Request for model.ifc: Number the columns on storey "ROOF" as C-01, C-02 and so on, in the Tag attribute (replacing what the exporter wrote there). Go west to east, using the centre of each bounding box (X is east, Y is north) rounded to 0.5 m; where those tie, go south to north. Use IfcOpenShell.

First a look at what the model holds.

```python
import ifcopenshell
import ifcopenshell.util.element
import ifcopenshell.util.placement

model = ifcopenshell.open("model.ifc")
print(model.schema)
storey = next(s for s in model.by_type("IfcBuildingStorey") if s.Name == "ROOF")
columns = [e for e in ifcopenshell.util.element.get_decomposition(storey) if e.is_a("IfcColumn")]
for e in sorted(columns, key=lambda e: e.id()):
    origin = ifcopenshell.util.placement.get_local_placement(e.ObjectPlacement)[:3, 3]
    print(e.id(), e.Tag, e.Name, origin.round(2) + 0.0, sep=" | ")
```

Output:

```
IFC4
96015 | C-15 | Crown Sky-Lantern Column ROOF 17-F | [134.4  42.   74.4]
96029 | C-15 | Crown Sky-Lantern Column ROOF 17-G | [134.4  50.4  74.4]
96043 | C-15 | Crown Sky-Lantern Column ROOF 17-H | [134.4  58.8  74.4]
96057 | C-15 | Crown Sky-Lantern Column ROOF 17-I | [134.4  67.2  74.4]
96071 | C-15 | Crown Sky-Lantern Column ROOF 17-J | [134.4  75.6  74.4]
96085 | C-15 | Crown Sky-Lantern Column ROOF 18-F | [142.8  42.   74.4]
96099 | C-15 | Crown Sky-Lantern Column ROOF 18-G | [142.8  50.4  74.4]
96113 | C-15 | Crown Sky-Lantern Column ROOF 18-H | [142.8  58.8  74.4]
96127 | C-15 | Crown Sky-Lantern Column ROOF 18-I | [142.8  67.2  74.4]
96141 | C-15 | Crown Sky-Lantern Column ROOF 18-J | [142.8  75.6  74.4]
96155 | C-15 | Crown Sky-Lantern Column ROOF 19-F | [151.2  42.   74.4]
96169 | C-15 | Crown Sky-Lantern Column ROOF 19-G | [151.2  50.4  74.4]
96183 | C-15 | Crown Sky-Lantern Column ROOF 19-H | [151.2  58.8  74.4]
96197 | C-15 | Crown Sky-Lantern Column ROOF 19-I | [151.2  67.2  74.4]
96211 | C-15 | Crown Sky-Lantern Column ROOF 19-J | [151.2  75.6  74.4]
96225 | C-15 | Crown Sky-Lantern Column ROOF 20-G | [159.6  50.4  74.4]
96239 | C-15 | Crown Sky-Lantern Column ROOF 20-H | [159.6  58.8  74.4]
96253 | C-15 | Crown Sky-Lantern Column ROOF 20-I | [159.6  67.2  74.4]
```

```python
import ifcopenshell
import ifcopenshell.geom
import ifcopenshell.util.element
import ifcopenshell.util.shape

model = ifcopenshell.open("model.ifc")
settings = ifcopenshell.geom.settings()
settings.set("use-world-coords", True)


def centre(element):
    shape = ifcopenshell.geom.create_shape(settings, element)
    return ifcopenshell.util.shape.get_bbox_centroid(shape.geometry)


storey = next(s for s in model.by_type("IfcBuildingStorey") if s.Name == "ROOF")
columns = [e for e in ifcopenshell.util.element.get_decomposition(storey) if e.is_a("IfcColumn")]

# Insertion points can sit at a corner or the storey origin, so sort by the geometry (in metres).
centres = {e: centre(e) for e in columns}
columns.sort(key=lambda e: (round(centres[e][0] / 0.5), centres[e][1]))

for i, e in enumerate(columns, start=1):
    number = f"C-{i:02d}"
    e.Tag = number
    print(e.id(), number)

model.write("model_edited.ifc")
```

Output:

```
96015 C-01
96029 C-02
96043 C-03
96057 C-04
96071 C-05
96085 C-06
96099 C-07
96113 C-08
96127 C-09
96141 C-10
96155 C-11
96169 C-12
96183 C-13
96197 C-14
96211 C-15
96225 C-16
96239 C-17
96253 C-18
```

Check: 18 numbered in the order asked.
